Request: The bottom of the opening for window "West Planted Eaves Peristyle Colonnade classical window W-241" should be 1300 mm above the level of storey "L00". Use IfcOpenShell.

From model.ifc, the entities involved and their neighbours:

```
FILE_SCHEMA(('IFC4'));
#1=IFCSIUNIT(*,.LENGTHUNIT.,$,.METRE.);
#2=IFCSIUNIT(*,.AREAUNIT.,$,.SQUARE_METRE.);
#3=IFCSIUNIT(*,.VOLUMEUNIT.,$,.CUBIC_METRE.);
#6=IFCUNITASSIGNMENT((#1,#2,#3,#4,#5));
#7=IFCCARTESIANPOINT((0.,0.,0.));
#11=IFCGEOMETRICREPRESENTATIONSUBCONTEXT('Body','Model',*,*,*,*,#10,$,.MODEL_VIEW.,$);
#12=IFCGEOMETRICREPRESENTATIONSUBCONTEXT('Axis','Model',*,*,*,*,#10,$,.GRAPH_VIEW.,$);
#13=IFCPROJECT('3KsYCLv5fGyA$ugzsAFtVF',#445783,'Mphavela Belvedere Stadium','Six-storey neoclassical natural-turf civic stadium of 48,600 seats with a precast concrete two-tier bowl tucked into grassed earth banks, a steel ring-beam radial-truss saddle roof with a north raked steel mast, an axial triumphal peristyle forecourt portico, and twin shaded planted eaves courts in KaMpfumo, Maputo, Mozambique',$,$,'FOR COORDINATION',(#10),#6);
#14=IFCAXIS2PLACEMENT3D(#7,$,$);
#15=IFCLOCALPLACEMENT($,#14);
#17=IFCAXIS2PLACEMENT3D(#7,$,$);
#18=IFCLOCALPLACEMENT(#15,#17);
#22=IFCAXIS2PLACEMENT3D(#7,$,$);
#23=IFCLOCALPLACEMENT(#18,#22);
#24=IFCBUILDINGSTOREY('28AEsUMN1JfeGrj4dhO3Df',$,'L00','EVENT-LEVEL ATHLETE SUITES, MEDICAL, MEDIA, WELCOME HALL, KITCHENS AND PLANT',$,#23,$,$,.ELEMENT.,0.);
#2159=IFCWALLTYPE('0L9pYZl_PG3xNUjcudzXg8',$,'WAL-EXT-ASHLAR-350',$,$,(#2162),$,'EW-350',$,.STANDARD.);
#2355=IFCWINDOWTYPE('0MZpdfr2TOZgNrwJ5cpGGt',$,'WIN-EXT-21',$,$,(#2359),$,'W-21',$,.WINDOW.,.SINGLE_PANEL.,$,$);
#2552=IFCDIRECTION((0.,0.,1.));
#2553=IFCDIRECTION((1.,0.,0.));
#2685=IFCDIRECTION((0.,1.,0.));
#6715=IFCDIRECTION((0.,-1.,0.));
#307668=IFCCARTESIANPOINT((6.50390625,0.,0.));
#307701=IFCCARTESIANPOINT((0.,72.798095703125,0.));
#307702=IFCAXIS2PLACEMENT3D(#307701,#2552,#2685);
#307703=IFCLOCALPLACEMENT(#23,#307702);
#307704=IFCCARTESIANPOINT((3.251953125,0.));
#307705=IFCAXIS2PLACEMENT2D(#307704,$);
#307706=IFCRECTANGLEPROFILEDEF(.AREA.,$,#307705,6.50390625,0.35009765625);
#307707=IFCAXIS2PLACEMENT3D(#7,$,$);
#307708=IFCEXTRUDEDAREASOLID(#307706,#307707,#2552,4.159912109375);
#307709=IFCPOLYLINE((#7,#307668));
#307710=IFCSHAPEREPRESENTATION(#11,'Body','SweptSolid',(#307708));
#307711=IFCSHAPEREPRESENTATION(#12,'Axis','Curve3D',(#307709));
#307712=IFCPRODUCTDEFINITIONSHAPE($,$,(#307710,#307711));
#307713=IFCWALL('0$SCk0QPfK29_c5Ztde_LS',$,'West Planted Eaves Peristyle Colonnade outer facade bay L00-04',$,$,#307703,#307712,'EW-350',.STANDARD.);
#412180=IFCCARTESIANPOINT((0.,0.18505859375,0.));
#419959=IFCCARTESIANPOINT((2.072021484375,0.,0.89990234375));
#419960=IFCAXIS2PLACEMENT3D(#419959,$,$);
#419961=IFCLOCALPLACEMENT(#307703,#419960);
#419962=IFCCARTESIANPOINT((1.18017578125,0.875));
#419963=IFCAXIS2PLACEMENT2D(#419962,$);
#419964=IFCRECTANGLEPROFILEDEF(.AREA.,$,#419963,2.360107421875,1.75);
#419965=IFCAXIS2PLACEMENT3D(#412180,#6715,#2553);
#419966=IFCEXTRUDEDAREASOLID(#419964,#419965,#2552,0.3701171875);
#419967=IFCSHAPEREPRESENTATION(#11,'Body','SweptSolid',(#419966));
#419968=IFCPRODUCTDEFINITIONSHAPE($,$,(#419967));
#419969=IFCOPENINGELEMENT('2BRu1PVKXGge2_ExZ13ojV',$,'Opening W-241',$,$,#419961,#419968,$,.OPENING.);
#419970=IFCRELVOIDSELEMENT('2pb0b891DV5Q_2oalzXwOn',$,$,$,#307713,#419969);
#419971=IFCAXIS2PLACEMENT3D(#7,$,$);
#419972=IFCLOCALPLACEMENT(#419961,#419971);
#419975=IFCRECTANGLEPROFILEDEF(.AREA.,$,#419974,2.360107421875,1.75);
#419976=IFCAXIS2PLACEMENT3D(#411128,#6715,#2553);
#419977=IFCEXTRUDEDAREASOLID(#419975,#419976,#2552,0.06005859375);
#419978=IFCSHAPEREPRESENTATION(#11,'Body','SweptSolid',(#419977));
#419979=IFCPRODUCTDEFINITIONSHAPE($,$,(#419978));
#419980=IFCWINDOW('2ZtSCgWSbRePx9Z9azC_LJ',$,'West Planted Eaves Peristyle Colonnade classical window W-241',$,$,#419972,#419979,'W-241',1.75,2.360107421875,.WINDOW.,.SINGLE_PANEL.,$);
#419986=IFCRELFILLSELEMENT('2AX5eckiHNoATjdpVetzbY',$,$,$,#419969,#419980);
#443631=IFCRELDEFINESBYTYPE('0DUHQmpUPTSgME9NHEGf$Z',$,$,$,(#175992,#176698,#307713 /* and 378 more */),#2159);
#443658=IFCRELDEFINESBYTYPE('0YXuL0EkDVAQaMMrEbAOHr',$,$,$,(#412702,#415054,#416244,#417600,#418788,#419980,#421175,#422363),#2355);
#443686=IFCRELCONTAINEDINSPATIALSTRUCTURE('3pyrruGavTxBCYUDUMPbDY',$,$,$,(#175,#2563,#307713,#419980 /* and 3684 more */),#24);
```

```python
import numpy as np
import ifcopenshell
import ifcopenshell.api.geometry
import ifcopenshell.geom
import ifcopenshell.util.element
import ifcopenshell.util.placement
import ifcopenshell.util.shape
import ifcopenshell.util.unit

model = ifcopenshell.open("model.ifc")
unit_scale = ifcopenshell.util.unit.calculate_unit_scale(model)

window = model.by_guid("2ZtSCgWSbRePx9Z9azC_LJ")
opening = window.FillsVoids[0].RelatingOpeningElement
storey = ifcopenshell.util.element.get_container(window, ifc_class="IfcBuildingStorey")
level = ifcopenshell.util.placement.get_local_placement(storey.ObjectPlacement)[2, 3]

# The opening's origin need not be at the sill, so measure its lowest point.
shape = ifcopenshell.geom.create_shape(ifcopenshell.geom.settings(), opening)
bottom = ifcopenshell.util.shape.get_shape_bottom_elevation(shape, shape.geometry) / unit_scale
dz = level + 1.3 / unit_scale - bottom

shift = np.array([0.0, 0.0, dz])
# The window is placed relative to its opening, so it follows when the opening moves.
matrix = ifcopenshell.util.placement.get_local_placement(opening.ObjectPlacement)
matrix[:3, 3] += shift
ifcopenshell.api.geometry.edit_object_placement(
    model, product=opening, matrix=matrix, is_si=False, should_transform_children=True
)

print(f"moved by {dz * unit_scale:+.3f} m")

model.write("model_edited.ifc")
```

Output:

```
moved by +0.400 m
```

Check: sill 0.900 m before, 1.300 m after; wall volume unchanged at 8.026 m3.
